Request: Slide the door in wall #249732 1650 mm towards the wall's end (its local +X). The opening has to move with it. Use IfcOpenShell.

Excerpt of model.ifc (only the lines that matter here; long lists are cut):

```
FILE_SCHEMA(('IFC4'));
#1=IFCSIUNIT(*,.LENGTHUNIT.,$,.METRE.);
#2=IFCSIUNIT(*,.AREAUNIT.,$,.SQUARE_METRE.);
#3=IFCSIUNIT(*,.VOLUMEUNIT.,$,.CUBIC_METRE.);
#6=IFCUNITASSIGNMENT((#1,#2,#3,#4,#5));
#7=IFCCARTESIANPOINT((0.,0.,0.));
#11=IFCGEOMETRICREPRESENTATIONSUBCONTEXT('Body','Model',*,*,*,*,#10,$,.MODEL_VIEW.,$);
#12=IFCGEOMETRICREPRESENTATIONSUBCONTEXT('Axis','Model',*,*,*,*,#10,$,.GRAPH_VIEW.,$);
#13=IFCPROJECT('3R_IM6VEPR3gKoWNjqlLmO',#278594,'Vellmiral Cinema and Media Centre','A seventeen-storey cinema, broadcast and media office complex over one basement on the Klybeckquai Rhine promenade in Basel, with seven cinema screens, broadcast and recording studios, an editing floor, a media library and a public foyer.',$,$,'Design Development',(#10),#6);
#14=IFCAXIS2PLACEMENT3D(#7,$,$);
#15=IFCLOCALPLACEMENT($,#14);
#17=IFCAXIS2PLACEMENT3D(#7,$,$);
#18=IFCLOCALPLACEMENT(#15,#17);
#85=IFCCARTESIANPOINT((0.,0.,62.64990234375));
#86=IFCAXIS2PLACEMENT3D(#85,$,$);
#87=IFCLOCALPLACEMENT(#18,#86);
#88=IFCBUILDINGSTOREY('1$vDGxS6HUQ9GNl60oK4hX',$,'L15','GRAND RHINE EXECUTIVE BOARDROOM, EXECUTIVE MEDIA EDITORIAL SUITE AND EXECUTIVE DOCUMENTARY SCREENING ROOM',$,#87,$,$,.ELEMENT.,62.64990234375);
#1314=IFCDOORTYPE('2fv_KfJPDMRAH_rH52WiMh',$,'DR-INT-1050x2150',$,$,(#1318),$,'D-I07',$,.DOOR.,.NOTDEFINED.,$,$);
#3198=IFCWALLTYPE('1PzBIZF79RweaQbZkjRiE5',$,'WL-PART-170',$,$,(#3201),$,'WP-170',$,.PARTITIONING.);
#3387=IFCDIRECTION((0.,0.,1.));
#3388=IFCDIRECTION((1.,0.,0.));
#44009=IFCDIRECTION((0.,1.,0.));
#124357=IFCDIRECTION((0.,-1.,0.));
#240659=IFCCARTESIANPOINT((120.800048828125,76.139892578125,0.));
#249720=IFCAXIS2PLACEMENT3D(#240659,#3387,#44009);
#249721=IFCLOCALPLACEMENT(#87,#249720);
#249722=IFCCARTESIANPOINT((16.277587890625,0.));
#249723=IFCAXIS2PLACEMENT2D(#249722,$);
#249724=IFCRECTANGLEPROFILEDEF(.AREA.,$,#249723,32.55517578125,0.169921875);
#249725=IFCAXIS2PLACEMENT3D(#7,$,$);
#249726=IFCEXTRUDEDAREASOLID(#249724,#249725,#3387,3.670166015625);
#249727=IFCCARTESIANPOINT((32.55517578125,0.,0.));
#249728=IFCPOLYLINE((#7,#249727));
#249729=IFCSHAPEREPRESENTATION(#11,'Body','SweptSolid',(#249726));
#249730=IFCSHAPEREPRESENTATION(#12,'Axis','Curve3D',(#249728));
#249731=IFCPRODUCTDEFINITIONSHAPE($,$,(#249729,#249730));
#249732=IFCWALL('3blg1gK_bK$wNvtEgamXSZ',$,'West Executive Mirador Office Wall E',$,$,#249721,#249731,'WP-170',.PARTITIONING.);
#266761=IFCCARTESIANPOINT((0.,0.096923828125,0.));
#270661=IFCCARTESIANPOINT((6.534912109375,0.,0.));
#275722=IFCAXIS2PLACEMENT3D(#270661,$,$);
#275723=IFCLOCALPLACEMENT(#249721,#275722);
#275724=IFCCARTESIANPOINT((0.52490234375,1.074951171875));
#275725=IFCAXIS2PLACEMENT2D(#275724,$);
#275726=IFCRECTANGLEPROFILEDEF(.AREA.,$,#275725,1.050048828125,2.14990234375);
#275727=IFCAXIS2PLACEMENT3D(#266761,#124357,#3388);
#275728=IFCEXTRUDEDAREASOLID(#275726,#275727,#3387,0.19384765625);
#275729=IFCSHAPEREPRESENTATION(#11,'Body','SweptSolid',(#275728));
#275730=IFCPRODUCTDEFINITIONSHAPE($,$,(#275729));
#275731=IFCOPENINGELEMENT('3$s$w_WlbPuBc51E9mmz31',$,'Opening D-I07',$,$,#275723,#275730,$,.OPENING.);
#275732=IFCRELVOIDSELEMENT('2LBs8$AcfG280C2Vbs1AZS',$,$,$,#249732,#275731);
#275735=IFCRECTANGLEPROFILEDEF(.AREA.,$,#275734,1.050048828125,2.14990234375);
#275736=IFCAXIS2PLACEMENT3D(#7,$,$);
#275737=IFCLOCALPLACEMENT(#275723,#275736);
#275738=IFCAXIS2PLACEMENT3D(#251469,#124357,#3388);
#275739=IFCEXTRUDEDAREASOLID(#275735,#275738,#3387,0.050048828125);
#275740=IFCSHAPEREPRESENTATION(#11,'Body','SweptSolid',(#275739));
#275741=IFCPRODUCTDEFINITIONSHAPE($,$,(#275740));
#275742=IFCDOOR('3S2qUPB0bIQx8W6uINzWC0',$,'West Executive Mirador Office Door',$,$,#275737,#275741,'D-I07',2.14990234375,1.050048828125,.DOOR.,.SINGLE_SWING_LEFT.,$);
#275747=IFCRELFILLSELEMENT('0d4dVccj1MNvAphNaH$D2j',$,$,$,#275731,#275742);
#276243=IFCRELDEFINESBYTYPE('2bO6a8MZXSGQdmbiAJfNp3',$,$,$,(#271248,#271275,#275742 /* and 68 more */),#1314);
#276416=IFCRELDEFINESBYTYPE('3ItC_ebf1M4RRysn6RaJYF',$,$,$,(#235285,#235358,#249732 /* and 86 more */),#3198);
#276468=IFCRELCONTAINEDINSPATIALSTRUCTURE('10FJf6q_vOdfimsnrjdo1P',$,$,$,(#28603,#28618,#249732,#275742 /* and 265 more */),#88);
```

```python
import ifcopenshell
import ifcopenshell.api.geometry
import ifcopenshell.util.placement

model = ifcopenshell.open("model.ifc")

door = model.by_guid("3S2qUPB0bIQx8W6uINzWC0")
opening = door.FillsVoids[0].RelatingOpeningElement
wall = opening.VoidsElements[0].RelatingBuildingElement

wall_matrix = ifcopenshell.util.placement.get_local_placement(wall.ObjectPlacement)
shift = wall_matrix[:3, 0] * 1.65
before = ifcopenshell.util.placement.get_local_placement(door.ObjectPlacement)[:3, 3].copy()

# The door is placed relative to its opening, so it follows when the opening moves.
matrix = ifcopenshell.util.placement.get_local_placement(opening.ObjectPlacement)
matrix[:3, 3] += shift
ifcopenshell.api.geometry.edit_object_placement(
    model, product=opening, matrix=matrix, is_si=False, should_transform_children=True
)

after = ifcopenshell.util.placement.get_local_placement(door.ObjectPlacement)[:3, 3]
print("door moved by", (after - before).round(3) + 0.0)

model.write("model_v2.ifc")
```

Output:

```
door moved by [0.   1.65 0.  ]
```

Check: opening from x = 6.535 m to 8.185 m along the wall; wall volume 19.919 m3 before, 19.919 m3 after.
